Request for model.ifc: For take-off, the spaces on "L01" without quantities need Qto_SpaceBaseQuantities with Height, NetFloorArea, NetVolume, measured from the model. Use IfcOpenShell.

First a look at what the model holds.

```python
import ifcopenshell
import ifcopenshell.util.element
import ifcopenshell.util.unit

model = ifcopenshell.open("model.ifc")
print(model.schema)
for unit_type in ("LENGTHUNIT", "AREAUNIT", "VOLUMEUNIT"):
    print(unit_type, ifcopenshell.util.unit.calculate_unit_scale(model, unit_type))
storey = next(s for s in model.by_type("IfcBuildingStorey") if s.Name == "L01")
spaces = [e for e in ifcopenshell.util.element.get_decomposition(storey) if e.is_a("IfcSpace")]
for e in sorted(spaces, key=lambda e: e.id()):
    print(e.id(), e.is_a(), e.Name, list(ifcopenshell.util.element.get_psets(e, qtos_only=True)), sep=" | ")
```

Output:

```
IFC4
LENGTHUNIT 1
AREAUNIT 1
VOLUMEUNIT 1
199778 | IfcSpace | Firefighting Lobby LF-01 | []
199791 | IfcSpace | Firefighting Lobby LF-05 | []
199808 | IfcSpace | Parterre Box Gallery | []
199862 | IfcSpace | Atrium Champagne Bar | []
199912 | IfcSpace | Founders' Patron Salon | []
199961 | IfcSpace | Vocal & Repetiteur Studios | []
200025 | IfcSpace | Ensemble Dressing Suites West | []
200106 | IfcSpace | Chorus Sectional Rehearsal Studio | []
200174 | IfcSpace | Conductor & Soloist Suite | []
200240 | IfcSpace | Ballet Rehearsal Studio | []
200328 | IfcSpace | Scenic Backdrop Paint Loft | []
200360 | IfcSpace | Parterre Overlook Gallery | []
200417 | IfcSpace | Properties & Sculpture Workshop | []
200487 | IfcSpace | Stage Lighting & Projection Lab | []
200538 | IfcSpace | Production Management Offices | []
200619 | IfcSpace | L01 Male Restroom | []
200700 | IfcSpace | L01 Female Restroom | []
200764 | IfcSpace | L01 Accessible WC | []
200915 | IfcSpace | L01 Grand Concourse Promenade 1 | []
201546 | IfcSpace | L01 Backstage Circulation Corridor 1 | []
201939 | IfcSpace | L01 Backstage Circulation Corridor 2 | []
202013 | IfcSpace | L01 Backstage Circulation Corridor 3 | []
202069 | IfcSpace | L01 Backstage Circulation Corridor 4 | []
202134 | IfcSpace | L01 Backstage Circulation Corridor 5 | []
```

```python
import ifcopenshell
import ifcopenshell.api.pset
import ifcopenshell.geom
import ifcopenshell.util.element
import ifcopenshell.util.shape
import ifcopenshell.util.unit

model = ifcopenshell.open("model.ifc")
unit_scale = ifcopenshell.util.unit.calculate_unit_scale(model)
area_scale = ifcopenshell.util.unit.calculate_unit_scale(model, "AREAUNIT")
volume_scale = ifcopenshell.util.unit.calculate_unit_scale(model, "VOLUMEUNIT")
settings = ifcopenshell.geom.settings()

storey = next(s for s in model.by_type("IfcBuildingStorey") if s.Name == "L01")
spaces = [e for e in ifcopenshell.util.element.get_decomposition(storey) if e.is_a("IfcSpace")]

for e in sorted(spaces, key=lambda e: e.id()):
    if ifcopenshell.util.element.get_psets(e, qtos_only=True, should_inherit=False):
        continue
    # Geometry comes back in metres, in the element's own axes.
    shape = ifcopenshell.geom.create_shape(settings, e)
    values = {
        "Height": ifcopenshell.util.shape.get_z(shape.geometry) / unit_scale,
        "NetFloorArea": ifcopenshell.util.shape.get_footprint_area(shape.geometry) / area_scale,
        "NetVolume": ifcopenshell.util.shape.get_volume(shape.geometry) / volume_scale,
    }
    qto = ifcopenshell.api.pset.add_qto(model, product=e, name="Qto_SpaceBaseQuantities")
    ifcopenshell.api.pset.edit_qto(model, qto=qto, properties=values)
    print(e.id(), {k: round(v, 3) for k, v in values.items()})

model.write("model_edited.ifc")
```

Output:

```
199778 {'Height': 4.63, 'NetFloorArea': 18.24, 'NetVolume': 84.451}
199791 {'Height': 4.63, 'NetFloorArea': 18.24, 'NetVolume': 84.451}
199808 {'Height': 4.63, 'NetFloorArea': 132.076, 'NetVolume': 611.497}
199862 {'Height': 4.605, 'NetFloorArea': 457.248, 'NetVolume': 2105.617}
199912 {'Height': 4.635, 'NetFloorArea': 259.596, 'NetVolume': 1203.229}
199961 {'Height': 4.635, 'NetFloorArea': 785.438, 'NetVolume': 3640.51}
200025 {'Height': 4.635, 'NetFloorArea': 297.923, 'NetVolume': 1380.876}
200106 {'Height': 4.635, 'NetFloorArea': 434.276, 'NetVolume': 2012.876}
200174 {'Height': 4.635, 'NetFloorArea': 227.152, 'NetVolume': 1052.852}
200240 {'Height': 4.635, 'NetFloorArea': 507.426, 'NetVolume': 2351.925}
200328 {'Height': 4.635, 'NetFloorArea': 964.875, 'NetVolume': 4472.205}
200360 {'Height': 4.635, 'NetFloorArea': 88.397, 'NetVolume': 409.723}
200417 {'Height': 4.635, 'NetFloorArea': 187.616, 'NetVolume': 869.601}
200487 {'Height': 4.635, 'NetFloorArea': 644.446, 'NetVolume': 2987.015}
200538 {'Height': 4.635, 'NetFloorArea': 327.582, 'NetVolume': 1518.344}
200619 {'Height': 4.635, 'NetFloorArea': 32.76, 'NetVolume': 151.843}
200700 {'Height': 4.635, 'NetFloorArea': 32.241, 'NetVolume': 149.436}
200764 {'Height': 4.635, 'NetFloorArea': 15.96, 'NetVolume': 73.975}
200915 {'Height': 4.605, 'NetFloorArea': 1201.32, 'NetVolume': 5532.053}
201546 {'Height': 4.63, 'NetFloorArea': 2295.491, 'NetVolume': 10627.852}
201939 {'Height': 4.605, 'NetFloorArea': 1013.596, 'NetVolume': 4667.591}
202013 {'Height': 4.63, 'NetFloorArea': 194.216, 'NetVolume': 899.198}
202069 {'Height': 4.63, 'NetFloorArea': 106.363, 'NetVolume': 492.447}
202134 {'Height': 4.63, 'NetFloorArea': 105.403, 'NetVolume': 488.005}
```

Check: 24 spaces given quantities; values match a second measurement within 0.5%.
